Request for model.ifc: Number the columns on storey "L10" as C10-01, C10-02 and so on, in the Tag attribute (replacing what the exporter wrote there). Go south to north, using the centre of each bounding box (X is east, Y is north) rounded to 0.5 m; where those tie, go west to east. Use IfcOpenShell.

First a look at what the model holds.

```python
import ifcopenshell
import ifcopenshell.util.element
import ifcopenshell.util.placement

model = ifcopenshell.open("model.ifc")
print(model.schema)
storey = next(s for s in model.by_type("IfcBuildingStorey") if s.Name == "L10")
columns = [e for e in ifcopenshell.util.element.get_decomposition(storey) if e.is_a("IfcColumn")]
for e in sorted(columns, key=lambda e: e.id()):
    origin = ifcopenshell.util.placement.get_local_placement(e.ObjectPlacement)[:3, 3]
    print(e.id(), e.Tag, e.Name, origin.round(2) + 0.0, sep=" | ")
```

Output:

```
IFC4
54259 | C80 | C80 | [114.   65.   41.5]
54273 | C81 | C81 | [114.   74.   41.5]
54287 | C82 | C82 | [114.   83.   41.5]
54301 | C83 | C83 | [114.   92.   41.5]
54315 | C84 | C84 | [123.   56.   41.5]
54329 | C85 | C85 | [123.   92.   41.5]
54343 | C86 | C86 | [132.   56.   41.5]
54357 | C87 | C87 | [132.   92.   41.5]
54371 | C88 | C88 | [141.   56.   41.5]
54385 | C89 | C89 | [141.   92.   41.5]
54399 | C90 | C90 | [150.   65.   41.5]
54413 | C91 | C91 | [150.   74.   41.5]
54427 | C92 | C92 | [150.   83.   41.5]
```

```python
import ifcopenshell
import ifcopenshell.geom
import ifcopenshell.util.element
import ifcopenshell.util.shape

model = ifcopenshell.open("model.ifc")
settings = ifcopenshell.geom.settings()
settings.set("use-world-coords", True)


def centre(element):
    shape = ifcopenshell.geom.create_shape(settings, element)
    return ifcopenshell.util.shape.get_bbox_centroid(shape.geometry)


storey = next(s for s in model.by_type("IfcBuildingStorey") if s.Name == "L10")
columns = [e for e in ifcopenshell.util.element.get_decomposition(storey) if e.is_a("IfcColumn")]

# Insertion points can sit at a corner or the storey origin, so sort by the geometry (in metres).
centres = {e: centre(e) for e in columns}
columns.sort(key=lambda e: (round(centres[e][1] / 0.5), centres[e][0]))

for i, e in enumerate(columns, start=1):
    number = f"C10-{i:02d}"
    e.Tag = number
    print(e.id(), number)

model.write("model_updated.ifc")
```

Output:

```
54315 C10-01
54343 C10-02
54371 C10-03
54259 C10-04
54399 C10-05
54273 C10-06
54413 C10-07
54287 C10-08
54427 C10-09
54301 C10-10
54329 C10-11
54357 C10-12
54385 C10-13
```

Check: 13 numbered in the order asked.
